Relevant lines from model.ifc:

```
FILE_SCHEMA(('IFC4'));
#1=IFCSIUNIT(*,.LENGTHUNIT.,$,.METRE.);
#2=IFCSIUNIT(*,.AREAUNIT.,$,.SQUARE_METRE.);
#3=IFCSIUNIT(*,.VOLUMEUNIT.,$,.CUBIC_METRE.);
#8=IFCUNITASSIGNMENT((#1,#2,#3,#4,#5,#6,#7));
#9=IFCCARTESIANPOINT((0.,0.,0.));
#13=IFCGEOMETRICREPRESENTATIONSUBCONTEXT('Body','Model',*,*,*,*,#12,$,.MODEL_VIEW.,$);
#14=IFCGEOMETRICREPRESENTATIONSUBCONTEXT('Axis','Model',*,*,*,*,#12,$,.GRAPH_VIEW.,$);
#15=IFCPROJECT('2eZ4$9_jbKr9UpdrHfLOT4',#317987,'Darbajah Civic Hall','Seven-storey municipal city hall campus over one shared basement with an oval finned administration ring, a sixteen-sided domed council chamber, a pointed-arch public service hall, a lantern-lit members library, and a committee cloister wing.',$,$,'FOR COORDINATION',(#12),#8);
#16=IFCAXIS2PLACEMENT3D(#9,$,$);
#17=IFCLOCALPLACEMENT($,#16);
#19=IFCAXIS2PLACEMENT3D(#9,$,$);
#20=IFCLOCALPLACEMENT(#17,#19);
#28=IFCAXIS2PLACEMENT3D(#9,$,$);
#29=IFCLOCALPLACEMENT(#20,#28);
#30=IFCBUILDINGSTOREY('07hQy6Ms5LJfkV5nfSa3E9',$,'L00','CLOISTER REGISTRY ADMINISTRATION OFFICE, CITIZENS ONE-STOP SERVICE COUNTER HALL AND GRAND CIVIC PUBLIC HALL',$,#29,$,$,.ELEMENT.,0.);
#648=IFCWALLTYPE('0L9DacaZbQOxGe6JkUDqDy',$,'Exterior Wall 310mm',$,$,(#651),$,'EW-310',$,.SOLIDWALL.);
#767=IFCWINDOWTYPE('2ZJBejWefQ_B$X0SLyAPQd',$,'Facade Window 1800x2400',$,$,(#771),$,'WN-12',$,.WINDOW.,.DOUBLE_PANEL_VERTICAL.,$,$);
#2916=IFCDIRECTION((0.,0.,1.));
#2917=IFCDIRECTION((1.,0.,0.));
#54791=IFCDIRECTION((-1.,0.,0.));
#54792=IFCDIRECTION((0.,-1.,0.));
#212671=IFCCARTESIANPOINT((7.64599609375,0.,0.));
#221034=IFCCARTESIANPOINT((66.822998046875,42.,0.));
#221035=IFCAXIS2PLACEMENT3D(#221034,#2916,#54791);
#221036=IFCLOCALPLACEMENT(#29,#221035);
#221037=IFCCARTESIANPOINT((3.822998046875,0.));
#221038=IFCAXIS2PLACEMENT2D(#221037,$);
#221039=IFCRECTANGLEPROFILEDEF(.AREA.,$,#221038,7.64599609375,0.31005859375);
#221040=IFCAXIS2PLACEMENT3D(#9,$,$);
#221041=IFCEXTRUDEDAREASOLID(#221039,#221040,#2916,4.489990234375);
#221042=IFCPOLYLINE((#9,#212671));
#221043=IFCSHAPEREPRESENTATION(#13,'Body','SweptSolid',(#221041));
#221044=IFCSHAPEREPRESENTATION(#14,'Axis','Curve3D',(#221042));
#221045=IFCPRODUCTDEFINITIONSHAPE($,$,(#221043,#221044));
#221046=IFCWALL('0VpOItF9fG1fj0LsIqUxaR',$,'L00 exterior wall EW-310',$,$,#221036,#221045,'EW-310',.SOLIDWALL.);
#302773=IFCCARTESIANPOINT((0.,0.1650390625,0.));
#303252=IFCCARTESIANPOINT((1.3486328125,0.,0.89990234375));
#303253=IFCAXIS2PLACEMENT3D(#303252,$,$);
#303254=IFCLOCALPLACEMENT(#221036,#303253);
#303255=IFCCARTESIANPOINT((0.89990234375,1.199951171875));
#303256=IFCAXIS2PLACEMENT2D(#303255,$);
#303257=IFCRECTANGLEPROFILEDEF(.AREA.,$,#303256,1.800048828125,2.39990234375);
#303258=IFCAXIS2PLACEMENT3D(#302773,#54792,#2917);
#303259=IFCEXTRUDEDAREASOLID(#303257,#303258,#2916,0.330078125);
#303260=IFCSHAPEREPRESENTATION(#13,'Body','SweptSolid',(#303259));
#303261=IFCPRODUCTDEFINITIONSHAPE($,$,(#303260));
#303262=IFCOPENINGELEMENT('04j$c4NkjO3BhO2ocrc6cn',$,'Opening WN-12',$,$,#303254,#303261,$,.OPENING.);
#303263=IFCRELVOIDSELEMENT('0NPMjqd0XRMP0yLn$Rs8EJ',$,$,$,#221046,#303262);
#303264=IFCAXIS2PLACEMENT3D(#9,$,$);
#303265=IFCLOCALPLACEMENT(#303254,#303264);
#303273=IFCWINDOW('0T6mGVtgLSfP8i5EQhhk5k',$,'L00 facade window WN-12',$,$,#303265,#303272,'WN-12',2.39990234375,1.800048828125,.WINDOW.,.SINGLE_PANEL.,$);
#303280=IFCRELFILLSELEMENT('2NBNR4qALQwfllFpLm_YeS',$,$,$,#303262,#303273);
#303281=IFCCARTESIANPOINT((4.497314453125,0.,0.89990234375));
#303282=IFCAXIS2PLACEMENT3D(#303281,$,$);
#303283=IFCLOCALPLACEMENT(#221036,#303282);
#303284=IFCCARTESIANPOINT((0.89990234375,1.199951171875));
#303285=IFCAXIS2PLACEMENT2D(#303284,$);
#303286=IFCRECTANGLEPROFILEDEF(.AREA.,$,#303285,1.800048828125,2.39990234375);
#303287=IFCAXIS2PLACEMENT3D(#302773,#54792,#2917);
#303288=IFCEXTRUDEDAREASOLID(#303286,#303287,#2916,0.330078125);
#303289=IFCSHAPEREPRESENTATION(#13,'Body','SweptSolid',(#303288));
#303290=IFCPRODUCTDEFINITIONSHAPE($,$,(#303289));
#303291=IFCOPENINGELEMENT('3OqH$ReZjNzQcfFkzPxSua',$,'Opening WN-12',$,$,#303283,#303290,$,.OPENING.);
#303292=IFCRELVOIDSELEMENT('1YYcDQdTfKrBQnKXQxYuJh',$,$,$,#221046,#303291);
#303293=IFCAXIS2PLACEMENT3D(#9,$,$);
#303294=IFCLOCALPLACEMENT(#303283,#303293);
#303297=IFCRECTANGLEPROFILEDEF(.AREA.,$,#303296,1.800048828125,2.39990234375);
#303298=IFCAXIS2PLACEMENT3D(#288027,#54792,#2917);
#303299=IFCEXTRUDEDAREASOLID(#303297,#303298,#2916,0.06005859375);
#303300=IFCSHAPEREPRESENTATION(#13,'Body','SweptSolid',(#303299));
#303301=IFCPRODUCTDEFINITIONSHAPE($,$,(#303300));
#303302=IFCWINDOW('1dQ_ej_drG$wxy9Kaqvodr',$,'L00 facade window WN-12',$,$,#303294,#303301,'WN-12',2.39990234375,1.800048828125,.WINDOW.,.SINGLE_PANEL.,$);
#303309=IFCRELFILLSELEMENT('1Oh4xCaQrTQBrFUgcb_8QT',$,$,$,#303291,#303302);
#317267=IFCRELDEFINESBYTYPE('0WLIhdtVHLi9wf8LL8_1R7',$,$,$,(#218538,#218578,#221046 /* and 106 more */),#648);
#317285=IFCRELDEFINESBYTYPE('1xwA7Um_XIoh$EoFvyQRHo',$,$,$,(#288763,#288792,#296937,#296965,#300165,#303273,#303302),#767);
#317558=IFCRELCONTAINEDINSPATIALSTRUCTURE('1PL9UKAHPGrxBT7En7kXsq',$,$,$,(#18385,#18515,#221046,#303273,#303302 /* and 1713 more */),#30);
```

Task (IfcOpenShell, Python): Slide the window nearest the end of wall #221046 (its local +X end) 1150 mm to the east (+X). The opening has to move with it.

```python
import ifcopenshell
import ifcopenshell.api.geometry
import ifcopenshell.util.placement
import ifcopenshell.util.unit

model = ifcopenshell.open("model.ifc")
unit_scale = ifcopenshell.util.unit.calculate_unit_scale(model)

window = model.by_guid("1dQ_ej_drG$wxy9Kaqvodr")
opening = window.FillsVoids[0].RelatingOpeningElement
wall = opening.VoidsElements[0].RelatingBuildingElement

wall_matrix = ifcopenshell.util.placement.get_local_placement(wall.ObjectPlacement)
shift = wall_matrix[:3, 0] * -1.15 / unit_scale
before = ifcopenshell.util.placement.get_local_placement(window.ObjectPlacement)[:3, 3].copy()

# The window is placed relative to its opening, so it follows when the opening moves.
matrix = ifcopenshell.util.placement.get_local_placement(opening.ObjectPlacement)
matrix[:3, 3] += shift
ifcopenshell.api.geometry.edit_object_placement(
    model, product=opening, matrix=matrix, is_si=False, should_transform_children=True
)

after = ifcopenshell.util.placement.get_local_placement(window.ObjectPlacement)[:3, 3]
print("window moved by", (after - before).round(3) + 0.0)

model.write("model_rev.ifc")
```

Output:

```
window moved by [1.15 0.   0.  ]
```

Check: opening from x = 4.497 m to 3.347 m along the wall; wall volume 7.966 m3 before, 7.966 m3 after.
